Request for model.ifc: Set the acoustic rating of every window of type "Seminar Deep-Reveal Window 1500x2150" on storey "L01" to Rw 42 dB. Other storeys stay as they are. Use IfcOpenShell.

First a look at what the model holds.

```python
import ifcopenshell
import ifcopenshell.util.element

model = ifcopenshell.open("model.ifc")
print(model.schema)
storey = next(s for s in model.by_type("IfcBuildingStorey") if s.Name == "L01")
windows = [e for e in ifcopenshell.util.element.get_decomposition(storey) if e.is_a("IfcWindow")]
seen = {}
for e in windows:
    element_type = ifcopenshell.util.element.get_type(e)
    key = (element_type.Name if element_type != e and element_type else None, ifcopenshell.util.element.get_pset(e, "Pset_WindowCommon", "AcousticRating"))
    seen[key] = seen.get(key, 0) + 1
for (name, value), count in sorted(seen.items(), key=str):
    print(count, "x", name, "|", value)
```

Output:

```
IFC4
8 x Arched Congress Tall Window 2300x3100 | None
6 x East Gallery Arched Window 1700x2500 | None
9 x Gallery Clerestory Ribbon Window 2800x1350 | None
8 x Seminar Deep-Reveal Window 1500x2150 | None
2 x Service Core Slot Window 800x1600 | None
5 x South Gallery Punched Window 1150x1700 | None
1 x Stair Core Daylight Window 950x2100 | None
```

```python
import ifcopenshell
import ifcopenshell.api.pset
import ifcopenshell.util.element

model = ifcopenshell.open("model.ifc")

storey = next(s for s in model.by_type("IfcBuildingStorey") if s.Name == "L01")
windows = [e for e in ifcopenshell.util.element.get_decomposition(storey) if e.is_a("IfcWindow")]

count = 0
for e in windows:
    element_type = ifcopenshell.util.element.get_type(e)
    if element_type in (None, e) or element_type.Name != "Seminar Deep-Reveal Window 1500x2150":
        continue
    # add_pset returns the element's existing set when there is one.
    pset = ifcopenshell.api.pset.add_pset(model, product=e, name="Pset_WindowCommon")
    ifcopenshell.api.pset.edit_pset(model, pset=pset, properties={"AcousticRating": "Rw 42 dB"})
    count += 1

print(count, "windows updated")

model.write("model_v2.ifc")
```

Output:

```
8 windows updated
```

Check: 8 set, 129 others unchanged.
